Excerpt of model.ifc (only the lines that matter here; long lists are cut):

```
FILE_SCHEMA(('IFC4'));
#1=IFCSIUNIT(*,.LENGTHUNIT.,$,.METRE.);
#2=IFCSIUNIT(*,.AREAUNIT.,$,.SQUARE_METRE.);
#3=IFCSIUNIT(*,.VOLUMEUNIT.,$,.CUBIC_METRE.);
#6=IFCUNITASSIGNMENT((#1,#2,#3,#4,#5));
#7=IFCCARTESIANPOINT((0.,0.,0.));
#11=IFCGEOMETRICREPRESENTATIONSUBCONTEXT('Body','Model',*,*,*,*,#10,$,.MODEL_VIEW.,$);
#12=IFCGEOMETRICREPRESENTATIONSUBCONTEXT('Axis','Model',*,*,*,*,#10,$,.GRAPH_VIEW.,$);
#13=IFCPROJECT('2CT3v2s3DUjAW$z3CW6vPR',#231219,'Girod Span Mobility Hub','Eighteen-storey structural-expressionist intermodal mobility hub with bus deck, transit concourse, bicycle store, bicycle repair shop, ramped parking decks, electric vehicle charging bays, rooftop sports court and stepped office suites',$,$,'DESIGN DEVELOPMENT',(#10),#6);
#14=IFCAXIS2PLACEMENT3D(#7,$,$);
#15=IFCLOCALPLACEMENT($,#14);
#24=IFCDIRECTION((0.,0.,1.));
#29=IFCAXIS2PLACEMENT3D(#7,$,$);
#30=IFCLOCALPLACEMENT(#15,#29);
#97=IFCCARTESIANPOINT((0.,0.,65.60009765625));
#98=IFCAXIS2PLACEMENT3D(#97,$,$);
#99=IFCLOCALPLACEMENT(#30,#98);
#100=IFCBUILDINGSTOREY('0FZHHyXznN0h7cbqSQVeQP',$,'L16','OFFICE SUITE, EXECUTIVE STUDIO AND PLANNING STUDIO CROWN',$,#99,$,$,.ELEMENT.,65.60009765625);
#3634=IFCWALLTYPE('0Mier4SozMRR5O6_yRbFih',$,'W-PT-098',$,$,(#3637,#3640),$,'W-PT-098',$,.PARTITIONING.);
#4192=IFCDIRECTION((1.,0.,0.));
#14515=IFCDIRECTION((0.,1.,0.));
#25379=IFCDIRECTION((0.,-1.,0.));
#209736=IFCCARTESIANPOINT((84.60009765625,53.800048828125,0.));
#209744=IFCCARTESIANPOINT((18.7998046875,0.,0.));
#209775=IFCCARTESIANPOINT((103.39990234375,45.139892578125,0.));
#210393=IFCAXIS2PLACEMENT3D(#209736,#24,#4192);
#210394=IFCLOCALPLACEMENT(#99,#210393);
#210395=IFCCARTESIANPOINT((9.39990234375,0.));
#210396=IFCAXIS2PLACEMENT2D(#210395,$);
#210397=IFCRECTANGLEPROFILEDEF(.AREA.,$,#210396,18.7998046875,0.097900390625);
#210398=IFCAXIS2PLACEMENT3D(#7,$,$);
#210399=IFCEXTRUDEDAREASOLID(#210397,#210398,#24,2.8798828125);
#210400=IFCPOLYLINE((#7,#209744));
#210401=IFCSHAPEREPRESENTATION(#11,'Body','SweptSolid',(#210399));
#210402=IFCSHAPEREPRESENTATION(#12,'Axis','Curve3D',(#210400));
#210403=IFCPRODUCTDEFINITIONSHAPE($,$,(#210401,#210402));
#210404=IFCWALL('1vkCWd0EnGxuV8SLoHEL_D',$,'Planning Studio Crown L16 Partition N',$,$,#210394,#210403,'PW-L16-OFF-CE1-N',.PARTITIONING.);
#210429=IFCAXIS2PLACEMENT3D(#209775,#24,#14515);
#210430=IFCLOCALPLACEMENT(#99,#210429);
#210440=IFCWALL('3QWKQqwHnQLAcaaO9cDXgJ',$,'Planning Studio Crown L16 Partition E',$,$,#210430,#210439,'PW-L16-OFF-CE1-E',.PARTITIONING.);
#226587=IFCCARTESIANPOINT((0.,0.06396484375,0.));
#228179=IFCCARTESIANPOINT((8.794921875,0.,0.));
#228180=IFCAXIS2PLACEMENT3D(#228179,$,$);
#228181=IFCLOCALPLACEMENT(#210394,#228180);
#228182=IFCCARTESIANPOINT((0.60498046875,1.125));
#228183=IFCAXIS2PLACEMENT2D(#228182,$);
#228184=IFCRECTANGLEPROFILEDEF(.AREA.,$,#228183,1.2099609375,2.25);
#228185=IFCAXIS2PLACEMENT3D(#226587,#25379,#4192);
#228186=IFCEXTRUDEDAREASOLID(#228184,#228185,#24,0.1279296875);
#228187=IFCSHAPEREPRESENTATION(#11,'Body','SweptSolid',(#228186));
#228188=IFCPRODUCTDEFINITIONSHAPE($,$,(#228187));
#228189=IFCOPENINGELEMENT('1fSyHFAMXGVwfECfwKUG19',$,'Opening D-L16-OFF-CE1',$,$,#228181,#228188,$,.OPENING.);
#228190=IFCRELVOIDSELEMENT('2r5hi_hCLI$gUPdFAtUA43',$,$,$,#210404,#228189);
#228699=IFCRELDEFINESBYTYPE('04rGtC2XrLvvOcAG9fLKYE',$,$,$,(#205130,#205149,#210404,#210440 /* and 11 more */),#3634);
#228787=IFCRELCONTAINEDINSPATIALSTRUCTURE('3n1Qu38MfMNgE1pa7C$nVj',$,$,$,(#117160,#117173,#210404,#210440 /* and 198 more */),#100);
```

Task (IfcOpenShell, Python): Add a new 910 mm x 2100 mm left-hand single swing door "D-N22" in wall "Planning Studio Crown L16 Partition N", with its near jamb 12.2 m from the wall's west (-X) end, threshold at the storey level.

```python
import numpy as np
import ifcopenshell
import ifcopenshell.api.feature
import ifcopenshell.api.geometry
import ifcopenshell.api.root
import ifcopenshell.api.spatial
import ifcopenshell.geom
import ifcopenshell.util.element
import ifcopenshell.util.placement
import ifcopenshell.util.representation
import ifcopenshell.util.shape
import ifcopenshell.util.unit

model = ifcopenshell.open("model.ifc")
unit_scale = ifcopenshell.util.unit.calculate_unit_scale(model)
settings = ifcopenshell.geom.settings()


def volume(element):
    """Net volume in cubic metres, openings subtracted."""
    shape = ifcopenshell.geom.create_shape(settings, element)
    return ifcopenshell.util.shape.get_volume(shape.geometry)


wall = model.by_id(210404)
storey = ifcopenshell.util.element.get_container(wall, ifc_class="IfcBuildingStorey")
context = ifcopenshell.util.representation.get_context(model, "Model", "Body", "MODEL_VIEW")
before = volume(wall)

width, height, from_end, sill = 0.91, 2.1, 12.2, 0.0  # metres

# The wall runs along its own X axis, and the end named is its -X end.
wall_shape = ifcopenshell.geom.create_shape(settings, wall)
x, y, z = ifcopenshell.util.shape.get_vertices(wall_shape.geometry).T
start = x.min() + from_end
face, thickness = float(y.min()), float(y.max() - y.min())
wall_matrix = ifcopenshell.util.placement.get_local_placement(wall.ObjectPlacement)
level = ifcopenshell.util.placement.get_local_placement(storey.ObjectPlacement)[2, 3]


def in_wall(x, y):
    """Placement at x, y metres in the wall's axes, at sill height."""
    matrix = wall_matrix.copy()
    matrix[:, 3] = wall_matrix @ np.array([x / unit_scale, y / unit_scale, 0.0, 1.0])
    matrix[2, 3] = level + sill / unit_scale
    return matrix


# Opening: a box that overshoots both wall faces by 50 mm.
opening = ifcopenshell.api.root.create_entity(model, ifc_class="IfcOpeningElement", predefined_type="OPENING")
box = ifcopenshell.api.geometry.add_wall_representation(
    model, context=context, length=width, height=height, thickness=thickness + 0.1
)
ifcopenshell.api.geometry.assign_representation(model, product=opening, representation=box)
ifcopenshell.api.geometry.edit_object_placement(model, product=opening, matrix=in_wall(start, face - 0.05), is_si=False)
ifcopenshell.api.feature.add_feature(model, feature=opening, element=wall)

door = ifcopenshell.api.root.create_entity(model, ifc_class="IfcDoor", name="D-N22", predefined_type="DOOR")
door.OverallWidth, door.OverallHeight = width / unit_scale, height / unit_scale
door.OperationType = "SINGLE_SWING_LEFT"
body = ifcopenshell.api.geometry.add_door_representation(
    model,
    context=context,
    overall_width=door.OverallWidth,
    overall_height=door.OverallHeight,
    operation_type="SINGLE_SWING_LEFT",
    lining_properties={"LiningDepth": thickness / unit_scale, "ThresholdDepth": thickness / unit_scale},
)
ifcopenshell.api.geometry.assign_representation(model, product=door, representation=body)
ifcopenshell.api.spatial.assign_container(model, products=[door], relating_structure=storey)
ifcopenshell.api.feature.add_filling(model, opening=opening, element=door)

# The lining spans the wall, so the door starts at the wall face.
ifcopenshell.api.geometry.edit_object_placement(model, product=door, matrix=in_wall(start, face), is_si=False)

after = volume(wall)

print(f"wall volume {before:.3f} -> {after:.3f} m3")

model.write("model_v2.ifc")
```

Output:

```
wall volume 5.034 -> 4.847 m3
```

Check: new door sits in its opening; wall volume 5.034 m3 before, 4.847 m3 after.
